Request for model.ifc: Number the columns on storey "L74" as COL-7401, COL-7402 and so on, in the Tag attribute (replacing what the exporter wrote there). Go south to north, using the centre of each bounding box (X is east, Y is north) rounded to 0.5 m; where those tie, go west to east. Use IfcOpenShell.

First a look at what the model holds.

```python
import ifcopenshell
import ifcopenshell.util.element
import ifcopenshell.util.placement

model = ifcopenshell.open("model.ifc")
print(model.schema)
storey = next(s for s in model.by_type("IfcBuildingStorey") if s.Name == "L74")
columns = [e for e in ifcopenshell.util.element.get_decomposition(storey) if e.is_a("IfcColumn")]
for e in sorted(columns, key=lambda e: e.id()):
    origin = ifcopenshell.util.placement.get_local_placement(e.ObjectPlacement)[:3, 3]
    print(e.id(), e.Tag, e.Name, origin.round(2) + 0.0, sep=" | ")
```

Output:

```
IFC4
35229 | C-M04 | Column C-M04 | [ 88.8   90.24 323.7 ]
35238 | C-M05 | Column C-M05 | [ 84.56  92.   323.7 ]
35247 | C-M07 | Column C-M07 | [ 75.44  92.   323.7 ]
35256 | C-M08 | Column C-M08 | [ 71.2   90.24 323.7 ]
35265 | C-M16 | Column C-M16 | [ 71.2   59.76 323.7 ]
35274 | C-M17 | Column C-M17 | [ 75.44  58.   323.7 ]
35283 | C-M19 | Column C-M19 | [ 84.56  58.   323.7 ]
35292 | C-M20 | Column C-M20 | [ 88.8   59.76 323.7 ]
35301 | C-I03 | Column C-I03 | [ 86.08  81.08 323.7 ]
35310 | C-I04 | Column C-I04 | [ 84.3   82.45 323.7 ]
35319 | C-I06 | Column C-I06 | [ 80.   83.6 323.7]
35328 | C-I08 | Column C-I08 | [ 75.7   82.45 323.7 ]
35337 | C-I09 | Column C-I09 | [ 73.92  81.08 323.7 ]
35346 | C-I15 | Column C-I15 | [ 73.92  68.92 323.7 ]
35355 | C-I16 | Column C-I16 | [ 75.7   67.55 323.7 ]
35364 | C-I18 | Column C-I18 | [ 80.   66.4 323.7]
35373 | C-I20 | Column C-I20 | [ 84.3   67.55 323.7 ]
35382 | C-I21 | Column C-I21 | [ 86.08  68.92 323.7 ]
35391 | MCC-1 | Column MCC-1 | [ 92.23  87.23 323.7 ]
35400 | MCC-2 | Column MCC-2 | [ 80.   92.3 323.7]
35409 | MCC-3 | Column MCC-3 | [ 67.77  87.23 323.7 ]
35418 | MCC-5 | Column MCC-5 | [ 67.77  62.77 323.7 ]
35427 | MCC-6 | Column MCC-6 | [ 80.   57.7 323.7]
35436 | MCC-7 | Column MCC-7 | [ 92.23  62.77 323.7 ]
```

```python
import ifcopenshell
import ifcopenshell.geom
import ifcopenshell.util.element
import ifcopenshell.util.shape

model = ifcopenshell.open("model.ifc")
settings = ifcopenshell.geom.settings()
settings.set("use-world-coords", True)


def centre(element):
    shape = ifcopenshell.geom.create_shape(settings, element)
    return ifcopenshell.util.shape.get_bbox_centroid(shape.geometry)


storey = next(s for s in model.by_type("IfcBuildingStorey") if s.Name == "L74")
columns = [e for e in ifcopenshell.util.element.get_decomposition(storey) if e.is_a("IfcColumn")]

# Insertion points can sit at a corner or the storey origin, so sort by the geometry (in metres).
centres = {e: centre(e) for e in columns}
columns.sort(key=lambda e: (round(centres[e][1] / 0.5), centres[e][0]))

for i, e in enumerate(columns, start=1):
    number = f"COL-74{i:02d}"
    e.Tag = number
    print(e.id(), number)

model.write("model_edited.ifc")
```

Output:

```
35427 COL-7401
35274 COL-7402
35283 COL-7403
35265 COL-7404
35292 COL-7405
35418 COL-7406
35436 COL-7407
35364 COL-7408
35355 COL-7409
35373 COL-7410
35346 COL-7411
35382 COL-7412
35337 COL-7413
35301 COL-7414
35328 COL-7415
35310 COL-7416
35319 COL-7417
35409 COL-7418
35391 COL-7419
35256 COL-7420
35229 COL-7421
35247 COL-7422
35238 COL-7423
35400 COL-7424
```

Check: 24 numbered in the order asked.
